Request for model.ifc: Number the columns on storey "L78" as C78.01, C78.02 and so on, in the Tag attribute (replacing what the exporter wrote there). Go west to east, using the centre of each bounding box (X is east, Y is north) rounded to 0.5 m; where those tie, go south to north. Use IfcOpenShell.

First a look at what the model holds.

```python
import ifcopenshell
import ifcopenshell.util.element
import ifcopenshell.util.placement

model = ifcopenshell.open("model.ifc")
print(model.schema)
storey = next(s for s in model.by_type("IfcBuildingStorey") if s.Name == "L78")
columns = [e for e in ifcopenshell.util.element.get_decomposition(storey) if e.is_a("IfcColumn")]
for e in sorted(columns, key=lambda e: e.id()):
    origin = ifcopenshell.util.placement.get_local_placement(e.ObjectPlacement)[:3, 3]
    print(e.id(), e.Tag, e.Name, origin.round(2) + 0.0, sep=" | ")
```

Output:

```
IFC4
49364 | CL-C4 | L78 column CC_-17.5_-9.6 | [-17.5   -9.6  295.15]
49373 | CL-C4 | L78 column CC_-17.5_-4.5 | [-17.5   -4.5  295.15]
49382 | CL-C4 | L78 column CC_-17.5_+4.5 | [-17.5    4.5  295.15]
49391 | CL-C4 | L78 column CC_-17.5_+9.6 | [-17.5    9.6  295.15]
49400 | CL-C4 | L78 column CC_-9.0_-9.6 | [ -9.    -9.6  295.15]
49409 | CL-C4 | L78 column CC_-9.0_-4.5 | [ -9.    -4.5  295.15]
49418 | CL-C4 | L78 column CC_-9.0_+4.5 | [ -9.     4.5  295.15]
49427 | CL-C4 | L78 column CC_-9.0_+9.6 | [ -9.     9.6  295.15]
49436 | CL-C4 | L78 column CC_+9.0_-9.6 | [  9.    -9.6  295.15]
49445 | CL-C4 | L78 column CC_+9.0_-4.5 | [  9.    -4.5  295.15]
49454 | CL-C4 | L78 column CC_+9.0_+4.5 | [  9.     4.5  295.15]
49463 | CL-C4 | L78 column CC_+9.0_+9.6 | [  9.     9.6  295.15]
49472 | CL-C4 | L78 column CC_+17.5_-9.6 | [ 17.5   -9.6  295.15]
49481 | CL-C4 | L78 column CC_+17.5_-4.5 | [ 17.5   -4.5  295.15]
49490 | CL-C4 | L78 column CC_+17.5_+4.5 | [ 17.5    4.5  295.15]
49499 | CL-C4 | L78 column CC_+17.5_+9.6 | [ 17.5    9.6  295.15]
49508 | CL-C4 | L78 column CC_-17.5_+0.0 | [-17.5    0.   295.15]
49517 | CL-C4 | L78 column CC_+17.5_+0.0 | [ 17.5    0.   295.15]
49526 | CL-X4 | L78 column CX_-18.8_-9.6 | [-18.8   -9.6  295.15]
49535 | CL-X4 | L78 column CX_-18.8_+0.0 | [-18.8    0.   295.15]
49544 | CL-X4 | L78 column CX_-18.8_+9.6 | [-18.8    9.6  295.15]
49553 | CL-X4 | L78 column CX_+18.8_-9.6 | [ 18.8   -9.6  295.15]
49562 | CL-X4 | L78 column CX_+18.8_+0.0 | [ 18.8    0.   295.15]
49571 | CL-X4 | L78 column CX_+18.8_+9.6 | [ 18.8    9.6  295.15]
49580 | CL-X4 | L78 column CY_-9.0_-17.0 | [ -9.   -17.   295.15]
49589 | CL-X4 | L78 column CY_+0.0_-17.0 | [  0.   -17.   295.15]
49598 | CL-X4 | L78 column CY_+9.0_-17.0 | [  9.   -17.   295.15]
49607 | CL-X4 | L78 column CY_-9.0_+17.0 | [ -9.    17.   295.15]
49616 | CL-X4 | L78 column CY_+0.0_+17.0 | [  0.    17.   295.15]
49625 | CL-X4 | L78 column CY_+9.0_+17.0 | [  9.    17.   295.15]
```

```python
import ifcopenshell
import ifcopenshell.geom
import ifcopenshell.util.element
import ifcopenshell.util.shape

model = ifcopenshell.open("model.ifc")
settings = ifcopenshell.geom.settings()
settings.set("use-world-coords", True)


def centre(element):
    shape = ifcopenshell.geom.create_shape(settings, element)
    return ifcopenshell.util.shape.get_bbox_centroid(shape.geometry)


storey = next(s for s in model.by_type("IfcBuildingStorey") if s.Name == "L78")
columns = [e for e in ifcopenshell.util.element.get_decomposition(storey) if e.is_a("IfcColumn")]

# Insertion points can sit at a corner or the storey origin, so sort by the geometry (in metres).
centres = {e: centre(e) for e in columns}
columns.sort(key=lambda e: (round(centres[e][0] / 0.5), centres[e][1]))

for i, e in enumerate(columns, start=1):
    number = f"C78.{i:02d}"
    e.Tag = number
    print(e.id(), number)

model.write("model_rev.ifc")
```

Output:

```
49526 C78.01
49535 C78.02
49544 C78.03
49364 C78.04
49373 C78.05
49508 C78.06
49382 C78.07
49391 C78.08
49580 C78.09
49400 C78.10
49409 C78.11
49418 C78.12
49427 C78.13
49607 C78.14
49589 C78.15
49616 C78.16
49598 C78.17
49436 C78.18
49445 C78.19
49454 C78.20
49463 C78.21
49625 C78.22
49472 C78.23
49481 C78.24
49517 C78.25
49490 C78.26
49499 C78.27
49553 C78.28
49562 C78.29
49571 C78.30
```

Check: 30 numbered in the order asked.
